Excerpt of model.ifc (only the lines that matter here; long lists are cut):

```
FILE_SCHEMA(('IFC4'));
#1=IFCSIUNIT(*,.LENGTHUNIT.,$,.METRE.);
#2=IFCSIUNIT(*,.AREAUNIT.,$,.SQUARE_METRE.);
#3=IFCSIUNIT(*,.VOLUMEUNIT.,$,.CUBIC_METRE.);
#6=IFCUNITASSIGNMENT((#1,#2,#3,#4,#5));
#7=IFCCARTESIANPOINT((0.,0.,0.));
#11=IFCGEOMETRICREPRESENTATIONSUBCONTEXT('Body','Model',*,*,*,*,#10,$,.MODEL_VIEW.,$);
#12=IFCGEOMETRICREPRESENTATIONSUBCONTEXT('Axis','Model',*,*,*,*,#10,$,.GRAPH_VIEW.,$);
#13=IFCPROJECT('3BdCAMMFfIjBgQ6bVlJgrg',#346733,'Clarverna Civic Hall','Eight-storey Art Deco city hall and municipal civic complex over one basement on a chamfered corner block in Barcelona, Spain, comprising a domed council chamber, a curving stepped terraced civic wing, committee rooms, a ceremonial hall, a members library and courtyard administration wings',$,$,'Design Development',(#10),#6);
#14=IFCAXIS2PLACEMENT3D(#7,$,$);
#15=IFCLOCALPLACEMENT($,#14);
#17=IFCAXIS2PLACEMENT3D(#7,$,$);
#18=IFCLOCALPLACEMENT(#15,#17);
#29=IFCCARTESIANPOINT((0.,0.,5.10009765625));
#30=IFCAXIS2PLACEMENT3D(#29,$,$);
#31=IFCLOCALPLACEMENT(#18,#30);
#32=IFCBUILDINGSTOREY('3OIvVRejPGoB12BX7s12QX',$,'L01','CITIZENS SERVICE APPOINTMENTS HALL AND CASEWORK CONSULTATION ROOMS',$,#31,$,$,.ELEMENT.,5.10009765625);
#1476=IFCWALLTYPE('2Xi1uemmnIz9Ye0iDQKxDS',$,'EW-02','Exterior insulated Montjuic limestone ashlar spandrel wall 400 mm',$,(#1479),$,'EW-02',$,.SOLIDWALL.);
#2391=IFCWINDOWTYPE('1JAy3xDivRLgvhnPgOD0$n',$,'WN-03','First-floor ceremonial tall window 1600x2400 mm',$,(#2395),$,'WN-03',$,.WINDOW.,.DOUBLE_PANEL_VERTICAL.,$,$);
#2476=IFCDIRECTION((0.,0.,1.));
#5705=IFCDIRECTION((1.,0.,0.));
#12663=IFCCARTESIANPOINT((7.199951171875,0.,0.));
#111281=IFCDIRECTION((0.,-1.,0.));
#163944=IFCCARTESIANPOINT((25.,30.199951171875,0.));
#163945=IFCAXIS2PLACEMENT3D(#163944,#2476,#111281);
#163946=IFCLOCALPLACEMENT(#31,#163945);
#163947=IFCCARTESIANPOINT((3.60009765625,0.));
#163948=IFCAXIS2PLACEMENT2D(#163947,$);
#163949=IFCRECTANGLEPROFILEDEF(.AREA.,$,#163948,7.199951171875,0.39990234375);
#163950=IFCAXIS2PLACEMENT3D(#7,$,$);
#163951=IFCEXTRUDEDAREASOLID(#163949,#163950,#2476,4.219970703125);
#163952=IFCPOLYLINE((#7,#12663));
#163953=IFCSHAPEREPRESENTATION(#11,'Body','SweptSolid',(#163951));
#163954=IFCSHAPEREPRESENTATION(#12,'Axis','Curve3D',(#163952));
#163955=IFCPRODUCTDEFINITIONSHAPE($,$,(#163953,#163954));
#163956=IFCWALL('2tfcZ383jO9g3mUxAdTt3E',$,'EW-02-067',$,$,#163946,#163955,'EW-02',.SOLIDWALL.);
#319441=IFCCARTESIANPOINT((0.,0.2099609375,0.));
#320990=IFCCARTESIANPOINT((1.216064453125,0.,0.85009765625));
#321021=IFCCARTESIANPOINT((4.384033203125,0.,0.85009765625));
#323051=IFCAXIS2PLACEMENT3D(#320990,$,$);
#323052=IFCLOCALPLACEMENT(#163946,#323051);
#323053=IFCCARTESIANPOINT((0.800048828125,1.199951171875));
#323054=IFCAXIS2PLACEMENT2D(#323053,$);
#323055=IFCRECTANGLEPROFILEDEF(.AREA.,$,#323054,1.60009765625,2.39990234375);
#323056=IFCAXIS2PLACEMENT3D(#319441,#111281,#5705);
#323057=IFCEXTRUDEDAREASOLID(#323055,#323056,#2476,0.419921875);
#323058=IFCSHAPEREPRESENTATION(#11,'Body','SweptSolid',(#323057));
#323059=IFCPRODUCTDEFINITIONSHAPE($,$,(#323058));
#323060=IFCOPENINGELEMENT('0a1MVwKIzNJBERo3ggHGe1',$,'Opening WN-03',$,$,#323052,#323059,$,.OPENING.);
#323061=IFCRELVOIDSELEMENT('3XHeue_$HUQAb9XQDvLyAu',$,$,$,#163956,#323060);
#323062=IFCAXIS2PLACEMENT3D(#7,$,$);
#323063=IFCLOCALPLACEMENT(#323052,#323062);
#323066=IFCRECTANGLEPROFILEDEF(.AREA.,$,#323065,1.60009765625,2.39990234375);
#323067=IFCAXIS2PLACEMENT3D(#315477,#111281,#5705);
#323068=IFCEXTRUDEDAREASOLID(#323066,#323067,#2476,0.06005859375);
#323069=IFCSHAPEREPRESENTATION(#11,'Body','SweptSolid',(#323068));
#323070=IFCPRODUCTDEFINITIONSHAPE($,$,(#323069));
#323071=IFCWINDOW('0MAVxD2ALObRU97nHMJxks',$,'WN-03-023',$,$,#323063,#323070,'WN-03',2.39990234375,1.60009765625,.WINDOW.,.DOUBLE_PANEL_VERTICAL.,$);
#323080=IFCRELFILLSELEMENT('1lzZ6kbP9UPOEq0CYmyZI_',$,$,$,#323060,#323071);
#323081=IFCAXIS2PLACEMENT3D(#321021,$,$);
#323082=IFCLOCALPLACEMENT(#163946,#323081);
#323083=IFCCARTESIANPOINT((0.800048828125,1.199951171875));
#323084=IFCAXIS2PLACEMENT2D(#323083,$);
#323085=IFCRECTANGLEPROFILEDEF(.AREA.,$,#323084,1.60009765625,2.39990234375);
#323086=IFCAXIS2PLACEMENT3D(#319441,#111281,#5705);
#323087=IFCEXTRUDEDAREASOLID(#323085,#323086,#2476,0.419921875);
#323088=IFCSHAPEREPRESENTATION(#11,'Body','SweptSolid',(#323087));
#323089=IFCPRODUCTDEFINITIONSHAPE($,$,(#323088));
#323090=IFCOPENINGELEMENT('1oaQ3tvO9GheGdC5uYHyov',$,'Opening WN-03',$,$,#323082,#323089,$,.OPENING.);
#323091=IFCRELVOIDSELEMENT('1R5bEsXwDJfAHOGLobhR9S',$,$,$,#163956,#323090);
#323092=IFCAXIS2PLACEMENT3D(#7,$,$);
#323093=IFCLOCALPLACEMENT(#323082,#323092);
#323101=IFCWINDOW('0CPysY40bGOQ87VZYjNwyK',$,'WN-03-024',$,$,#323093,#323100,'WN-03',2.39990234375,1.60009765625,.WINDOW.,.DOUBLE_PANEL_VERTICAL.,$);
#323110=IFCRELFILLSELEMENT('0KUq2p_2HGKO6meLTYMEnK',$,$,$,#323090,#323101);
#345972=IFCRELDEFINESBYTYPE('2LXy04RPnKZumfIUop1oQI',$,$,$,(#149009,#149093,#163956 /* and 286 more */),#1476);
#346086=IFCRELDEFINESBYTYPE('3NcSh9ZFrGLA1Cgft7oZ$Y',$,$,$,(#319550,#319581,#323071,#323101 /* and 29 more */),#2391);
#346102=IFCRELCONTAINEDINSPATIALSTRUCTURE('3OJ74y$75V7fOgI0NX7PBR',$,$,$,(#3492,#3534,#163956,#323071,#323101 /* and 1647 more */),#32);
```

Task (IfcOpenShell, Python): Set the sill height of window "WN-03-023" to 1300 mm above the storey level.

```python
import numpy as np
import ifcopenshell
import ifcopenshell.api.geometry
import ifcopenshell.geom
import ifcopenshell.util.element
import ifcopenshell.util.placement
import ifcopenshell.util.shape
import ifcopenshell.util.unit

model = ifcopenshell.open("model.ifc")
unit_scale = ifcopenshell.util.unit.calculate_unit_scale(model)

window = model.by_id(323071)
opening = window.FillsVoids[0].RelatingOpeningElement
storey = ifcopenshell.util.element.get_container(window, ifc_class="IfcBuildingStorey")
level = ifcopenshell.util.placement.get_local_placement(storey.ObjectPlacement)[2, 3]

# The opening's origin need not be at the sill, so measure its lowest point.
shape = ifcopenshell.geom.create_shape(ifcopenshell.geom.settings(), opening)
bottom = ifcopenshell.util.shape.get_shape_bottom_elevation(shape, shape.geometry) / unit_scale
dz = level + 1.3 / unit_scale - bottom

shift = np.array([0.0, 0.0, dz])
# The window is placed relative to its opening, so it follows when the opening moves.
matrix = ifcopenshell.util.placement.get_local_placement(opening.ObjectPlacement)
matrix[:3, 3] += shift
ifcopenshell.api.geometry.edit_object_placement(
    model, product=opening, matrix=matrix, is_si=False, should_transform_children=True
)

print(f"moved by {dz * unit_scale:+.3f} m")

model.write("model-out.ifc")
```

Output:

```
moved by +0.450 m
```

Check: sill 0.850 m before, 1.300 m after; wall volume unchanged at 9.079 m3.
